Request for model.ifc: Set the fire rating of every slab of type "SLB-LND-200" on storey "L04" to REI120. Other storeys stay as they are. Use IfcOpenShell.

First a look at what the model holds.

```python
import ifcopenshell
import ifcopenshell.util.element

model = ifcopenshell.open("model.ifc")
print(model.schema)
storey = next(s for s in model.by_type("IfcBuildingStorey") if s.Name == "L04")
slabs = [e for e in ifcopenshell.util.element.get_decomposition(storey) if e.is_a("IfcSlab")]
seen = {}
for e in slabs:
    element_type = ifcopenshell.util.element.get_type(e)
    key = (element_type.Name if element_type != e and element_type else None, ifcopenshell.util.element.get_pset(e, "Pset_SlabCommon", "FireRating"))
    seen[key] = seen.get(key, 0) + 1
for (name, value), count in sorted(seen.items(), key=str):
    print(count, "x", name, "|", value)
```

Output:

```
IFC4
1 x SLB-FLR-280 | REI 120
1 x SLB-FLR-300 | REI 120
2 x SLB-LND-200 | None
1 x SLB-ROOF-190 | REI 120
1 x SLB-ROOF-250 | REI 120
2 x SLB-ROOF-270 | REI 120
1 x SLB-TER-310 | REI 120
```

```python
import ifcopenshell
import ifcopenshell.api.pset
import ifcopenshell.util.element

model = ifcopenshell.open("model.ifc")

storey = next(s for s in model.by_type("IfcBuildingStorey") if s.Name == "L04")
slabs = [e for e in ifcopenshell.util.element.get_decomposition(storey) if e.is_a("IfcSlab")]

count = 0
for e in slabs:
    element_type = ifcopenshell.util.element.get_type(e)
    if element_type in (None, e) or element_type.Name != "SLB-LND-200":
        continue
    # add_pset returns the element's existing set when there is one.
    pset = ifcopenshell.api.pset.add_pset(model, product=e, name="Pset_SlabCommon")
    ifcopenshell.api.pset.edit_pset(model, pset=pset, properties={"FireRating": "REI120"})
    count += 1

print(count, "slabs updated")

model.write("model_v2.ifc")
```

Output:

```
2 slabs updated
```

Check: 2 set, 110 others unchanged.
